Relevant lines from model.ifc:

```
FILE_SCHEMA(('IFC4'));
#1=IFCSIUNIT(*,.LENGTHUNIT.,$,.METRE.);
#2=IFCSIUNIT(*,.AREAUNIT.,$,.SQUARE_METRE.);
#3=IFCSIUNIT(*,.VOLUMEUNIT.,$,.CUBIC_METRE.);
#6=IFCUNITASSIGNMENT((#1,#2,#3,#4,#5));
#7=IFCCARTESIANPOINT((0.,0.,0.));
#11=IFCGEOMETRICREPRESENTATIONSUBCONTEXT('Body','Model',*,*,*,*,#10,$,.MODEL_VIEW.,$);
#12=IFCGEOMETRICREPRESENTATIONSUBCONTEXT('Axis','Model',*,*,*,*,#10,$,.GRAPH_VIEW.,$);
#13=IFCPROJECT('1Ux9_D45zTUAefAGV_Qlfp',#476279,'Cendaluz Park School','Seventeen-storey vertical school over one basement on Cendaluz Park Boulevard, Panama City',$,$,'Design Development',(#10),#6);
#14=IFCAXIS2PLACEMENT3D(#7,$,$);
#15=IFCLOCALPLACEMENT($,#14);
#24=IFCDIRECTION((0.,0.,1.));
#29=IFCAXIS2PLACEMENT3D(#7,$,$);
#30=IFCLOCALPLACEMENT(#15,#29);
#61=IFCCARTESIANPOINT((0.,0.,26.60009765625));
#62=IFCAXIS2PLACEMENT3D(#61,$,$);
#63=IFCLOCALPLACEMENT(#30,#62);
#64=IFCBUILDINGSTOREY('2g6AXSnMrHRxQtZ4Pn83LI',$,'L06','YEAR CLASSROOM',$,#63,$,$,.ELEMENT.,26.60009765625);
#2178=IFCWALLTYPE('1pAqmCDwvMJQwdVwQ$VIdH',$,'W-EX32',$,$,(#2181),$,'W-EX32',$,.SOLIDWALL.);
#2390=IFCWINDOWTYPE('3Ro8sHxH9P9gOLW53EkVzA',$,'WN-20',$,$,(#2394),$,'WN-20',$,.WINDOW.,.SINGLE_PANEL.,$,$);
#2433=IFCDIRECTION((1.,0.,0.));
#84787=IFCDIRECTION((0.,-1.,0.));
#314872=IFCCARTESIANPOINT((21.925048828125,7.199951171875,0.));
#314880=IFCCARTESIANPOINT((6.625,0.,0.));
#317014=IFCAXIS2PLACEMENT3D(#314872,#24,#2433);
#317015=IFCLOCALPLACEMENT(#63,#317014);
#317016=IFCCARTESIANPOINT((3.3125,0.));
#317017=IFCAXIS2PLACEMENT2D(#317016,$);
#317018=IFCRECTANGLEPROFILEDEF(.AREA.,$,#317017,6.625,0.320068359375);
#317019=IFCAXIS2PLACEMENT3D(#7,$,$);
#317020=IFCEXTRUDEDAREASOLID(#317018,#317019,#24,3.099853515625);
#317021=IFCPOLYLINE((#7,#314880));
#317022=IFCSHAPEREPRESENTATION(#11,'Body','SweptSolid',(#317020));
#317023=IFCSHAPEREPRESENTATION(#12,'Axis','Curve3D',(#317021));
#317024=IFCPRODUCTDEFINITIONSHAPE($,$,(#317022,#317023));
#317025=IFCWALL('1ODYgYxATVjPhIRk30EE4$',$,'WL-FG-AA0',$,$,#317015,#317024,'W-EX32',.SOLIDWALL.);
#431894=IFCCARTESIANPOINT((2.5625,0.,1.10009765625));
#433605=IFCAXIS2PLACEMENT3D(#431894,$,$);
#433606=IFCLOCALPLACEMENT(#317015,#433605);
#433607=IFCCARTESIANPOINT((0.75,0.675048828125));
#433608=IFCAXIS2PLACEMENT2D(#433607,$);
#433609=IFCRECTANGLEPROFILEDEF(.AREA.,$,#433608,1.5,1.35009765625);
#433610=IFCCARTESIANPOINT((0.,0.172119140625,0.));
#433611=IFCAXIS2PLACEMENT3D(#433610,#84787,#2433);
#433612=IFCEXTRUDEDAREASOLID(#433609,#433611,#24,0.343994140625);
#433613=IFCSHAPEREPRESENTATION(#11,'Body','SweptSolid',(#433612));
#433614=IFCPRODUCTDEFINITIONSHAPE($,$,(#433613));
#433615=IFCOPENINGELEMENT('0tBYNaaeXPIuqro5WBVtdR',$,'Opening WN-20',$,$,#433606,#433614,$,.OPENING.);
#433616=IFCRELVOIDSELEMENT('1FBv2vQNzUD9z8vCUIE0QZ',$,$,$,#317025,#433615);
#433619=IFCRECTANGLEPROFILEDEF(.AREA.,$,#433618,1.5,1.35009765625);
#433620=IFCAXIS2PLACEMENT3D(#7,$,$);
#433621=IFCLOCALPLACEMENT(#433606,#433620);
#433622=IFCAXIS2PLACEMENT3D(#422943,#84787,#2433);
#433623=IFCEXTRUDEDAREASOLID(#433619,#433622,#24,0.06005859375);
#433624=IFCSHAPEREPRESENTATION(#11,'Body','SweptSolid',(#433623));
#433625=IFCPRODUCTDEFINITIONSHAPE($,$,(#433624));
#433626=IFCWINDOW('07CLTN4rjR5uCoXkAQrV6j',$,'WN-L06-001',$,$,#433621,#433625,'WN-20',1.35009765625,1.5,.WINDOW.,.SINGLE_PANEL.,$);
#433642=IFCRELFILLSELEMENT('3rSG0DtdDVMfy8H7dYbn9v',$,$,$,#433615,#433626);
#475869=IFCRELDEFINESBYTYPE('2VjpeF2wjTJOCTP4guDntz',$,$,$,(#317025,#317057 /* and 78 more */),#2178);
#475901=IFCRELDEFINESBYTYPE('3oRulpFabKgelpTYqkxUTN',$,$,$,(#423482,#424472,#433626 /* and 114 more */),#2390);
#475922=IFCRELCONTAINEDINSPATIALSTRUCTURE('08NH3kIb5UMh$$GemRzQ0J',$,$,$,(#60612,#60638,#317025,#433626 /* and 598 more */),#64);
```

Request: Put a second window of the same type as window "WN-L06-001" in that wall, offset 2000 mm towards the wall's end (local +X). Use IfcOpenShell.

```python
import ifcopenshell
import ifcopenshell.api.feature
import ifcopenshell.api.geometry
import ifcopenshell.api.root
import ifcopenshell.geom
import ifcopenshell.util.element
import ifcopenshell.util.placement
import ifcopenshell.util.shape

model = ifcopenshell.open("model.ifc")
settings = ifcopenshell.geom.settings()


def volume(element):
    """Net volume in cubic metres, openings subtracted."""
    shape = ifcopenshell.geom.create_shape(settings, element)
    return ifcopenshell.util.shape.get_volume(shape.geometry)


window = model.by_guid("07CLTN4rjR5uCoXkAQrV6j")
opening = window.FillsVoids[0].RelatingOpeningElement
wall = opening.VoidsElements[0].RelatingBuildingElement
before = volume(wall)
shift = ifcopenshell.util.placement.get_local_placement(wall.ObjectPlacement)[:3, 0] * 2.0

# copy_class copies the void relationship, type, container and properties, but no geometry.
new_opening = ifcopenshell.api.root.copy_class(model, product=opening)
new_opening.Representation = ifcopenshell.util.element.copy_deep(
    model, opening.Representation, exclude=["IfcGeometricRepresentationContext", "IfcRepresentationMap"]
)
new_window = ifcopenshell.api.root.copy_class(model, product=window)
new_window.Representation = ifcopenshell.util.element.copy_deep(
    model, window.Representation, exclude=["IfcGeometricRepresentationContext", "IfcRepresentationMap"]
)
new_window.Tag = None
ifcopenshell.api.feature.add_filling(model, opening=new_opening, element=new_window)

for old, new in ((opening, new_opening), (window, new_window)):
    matrix = ifcopenshell.util.placement.get_local_placement(old.ObjectPlacement)
    matrix[:3, 3] += shift
    ifcopenshell.api.geometry.edit_object_placement(model, product=new, matrix=matrix, is_si=False)

after = volume(wall)

print(f"wall volume {before:.3f} -> {after:.3f} m3")

model.write("model_edited.ifc")
```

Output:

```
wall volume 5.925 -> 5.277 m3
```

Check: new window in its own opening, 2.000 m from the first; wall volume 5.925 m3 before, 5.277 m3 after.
